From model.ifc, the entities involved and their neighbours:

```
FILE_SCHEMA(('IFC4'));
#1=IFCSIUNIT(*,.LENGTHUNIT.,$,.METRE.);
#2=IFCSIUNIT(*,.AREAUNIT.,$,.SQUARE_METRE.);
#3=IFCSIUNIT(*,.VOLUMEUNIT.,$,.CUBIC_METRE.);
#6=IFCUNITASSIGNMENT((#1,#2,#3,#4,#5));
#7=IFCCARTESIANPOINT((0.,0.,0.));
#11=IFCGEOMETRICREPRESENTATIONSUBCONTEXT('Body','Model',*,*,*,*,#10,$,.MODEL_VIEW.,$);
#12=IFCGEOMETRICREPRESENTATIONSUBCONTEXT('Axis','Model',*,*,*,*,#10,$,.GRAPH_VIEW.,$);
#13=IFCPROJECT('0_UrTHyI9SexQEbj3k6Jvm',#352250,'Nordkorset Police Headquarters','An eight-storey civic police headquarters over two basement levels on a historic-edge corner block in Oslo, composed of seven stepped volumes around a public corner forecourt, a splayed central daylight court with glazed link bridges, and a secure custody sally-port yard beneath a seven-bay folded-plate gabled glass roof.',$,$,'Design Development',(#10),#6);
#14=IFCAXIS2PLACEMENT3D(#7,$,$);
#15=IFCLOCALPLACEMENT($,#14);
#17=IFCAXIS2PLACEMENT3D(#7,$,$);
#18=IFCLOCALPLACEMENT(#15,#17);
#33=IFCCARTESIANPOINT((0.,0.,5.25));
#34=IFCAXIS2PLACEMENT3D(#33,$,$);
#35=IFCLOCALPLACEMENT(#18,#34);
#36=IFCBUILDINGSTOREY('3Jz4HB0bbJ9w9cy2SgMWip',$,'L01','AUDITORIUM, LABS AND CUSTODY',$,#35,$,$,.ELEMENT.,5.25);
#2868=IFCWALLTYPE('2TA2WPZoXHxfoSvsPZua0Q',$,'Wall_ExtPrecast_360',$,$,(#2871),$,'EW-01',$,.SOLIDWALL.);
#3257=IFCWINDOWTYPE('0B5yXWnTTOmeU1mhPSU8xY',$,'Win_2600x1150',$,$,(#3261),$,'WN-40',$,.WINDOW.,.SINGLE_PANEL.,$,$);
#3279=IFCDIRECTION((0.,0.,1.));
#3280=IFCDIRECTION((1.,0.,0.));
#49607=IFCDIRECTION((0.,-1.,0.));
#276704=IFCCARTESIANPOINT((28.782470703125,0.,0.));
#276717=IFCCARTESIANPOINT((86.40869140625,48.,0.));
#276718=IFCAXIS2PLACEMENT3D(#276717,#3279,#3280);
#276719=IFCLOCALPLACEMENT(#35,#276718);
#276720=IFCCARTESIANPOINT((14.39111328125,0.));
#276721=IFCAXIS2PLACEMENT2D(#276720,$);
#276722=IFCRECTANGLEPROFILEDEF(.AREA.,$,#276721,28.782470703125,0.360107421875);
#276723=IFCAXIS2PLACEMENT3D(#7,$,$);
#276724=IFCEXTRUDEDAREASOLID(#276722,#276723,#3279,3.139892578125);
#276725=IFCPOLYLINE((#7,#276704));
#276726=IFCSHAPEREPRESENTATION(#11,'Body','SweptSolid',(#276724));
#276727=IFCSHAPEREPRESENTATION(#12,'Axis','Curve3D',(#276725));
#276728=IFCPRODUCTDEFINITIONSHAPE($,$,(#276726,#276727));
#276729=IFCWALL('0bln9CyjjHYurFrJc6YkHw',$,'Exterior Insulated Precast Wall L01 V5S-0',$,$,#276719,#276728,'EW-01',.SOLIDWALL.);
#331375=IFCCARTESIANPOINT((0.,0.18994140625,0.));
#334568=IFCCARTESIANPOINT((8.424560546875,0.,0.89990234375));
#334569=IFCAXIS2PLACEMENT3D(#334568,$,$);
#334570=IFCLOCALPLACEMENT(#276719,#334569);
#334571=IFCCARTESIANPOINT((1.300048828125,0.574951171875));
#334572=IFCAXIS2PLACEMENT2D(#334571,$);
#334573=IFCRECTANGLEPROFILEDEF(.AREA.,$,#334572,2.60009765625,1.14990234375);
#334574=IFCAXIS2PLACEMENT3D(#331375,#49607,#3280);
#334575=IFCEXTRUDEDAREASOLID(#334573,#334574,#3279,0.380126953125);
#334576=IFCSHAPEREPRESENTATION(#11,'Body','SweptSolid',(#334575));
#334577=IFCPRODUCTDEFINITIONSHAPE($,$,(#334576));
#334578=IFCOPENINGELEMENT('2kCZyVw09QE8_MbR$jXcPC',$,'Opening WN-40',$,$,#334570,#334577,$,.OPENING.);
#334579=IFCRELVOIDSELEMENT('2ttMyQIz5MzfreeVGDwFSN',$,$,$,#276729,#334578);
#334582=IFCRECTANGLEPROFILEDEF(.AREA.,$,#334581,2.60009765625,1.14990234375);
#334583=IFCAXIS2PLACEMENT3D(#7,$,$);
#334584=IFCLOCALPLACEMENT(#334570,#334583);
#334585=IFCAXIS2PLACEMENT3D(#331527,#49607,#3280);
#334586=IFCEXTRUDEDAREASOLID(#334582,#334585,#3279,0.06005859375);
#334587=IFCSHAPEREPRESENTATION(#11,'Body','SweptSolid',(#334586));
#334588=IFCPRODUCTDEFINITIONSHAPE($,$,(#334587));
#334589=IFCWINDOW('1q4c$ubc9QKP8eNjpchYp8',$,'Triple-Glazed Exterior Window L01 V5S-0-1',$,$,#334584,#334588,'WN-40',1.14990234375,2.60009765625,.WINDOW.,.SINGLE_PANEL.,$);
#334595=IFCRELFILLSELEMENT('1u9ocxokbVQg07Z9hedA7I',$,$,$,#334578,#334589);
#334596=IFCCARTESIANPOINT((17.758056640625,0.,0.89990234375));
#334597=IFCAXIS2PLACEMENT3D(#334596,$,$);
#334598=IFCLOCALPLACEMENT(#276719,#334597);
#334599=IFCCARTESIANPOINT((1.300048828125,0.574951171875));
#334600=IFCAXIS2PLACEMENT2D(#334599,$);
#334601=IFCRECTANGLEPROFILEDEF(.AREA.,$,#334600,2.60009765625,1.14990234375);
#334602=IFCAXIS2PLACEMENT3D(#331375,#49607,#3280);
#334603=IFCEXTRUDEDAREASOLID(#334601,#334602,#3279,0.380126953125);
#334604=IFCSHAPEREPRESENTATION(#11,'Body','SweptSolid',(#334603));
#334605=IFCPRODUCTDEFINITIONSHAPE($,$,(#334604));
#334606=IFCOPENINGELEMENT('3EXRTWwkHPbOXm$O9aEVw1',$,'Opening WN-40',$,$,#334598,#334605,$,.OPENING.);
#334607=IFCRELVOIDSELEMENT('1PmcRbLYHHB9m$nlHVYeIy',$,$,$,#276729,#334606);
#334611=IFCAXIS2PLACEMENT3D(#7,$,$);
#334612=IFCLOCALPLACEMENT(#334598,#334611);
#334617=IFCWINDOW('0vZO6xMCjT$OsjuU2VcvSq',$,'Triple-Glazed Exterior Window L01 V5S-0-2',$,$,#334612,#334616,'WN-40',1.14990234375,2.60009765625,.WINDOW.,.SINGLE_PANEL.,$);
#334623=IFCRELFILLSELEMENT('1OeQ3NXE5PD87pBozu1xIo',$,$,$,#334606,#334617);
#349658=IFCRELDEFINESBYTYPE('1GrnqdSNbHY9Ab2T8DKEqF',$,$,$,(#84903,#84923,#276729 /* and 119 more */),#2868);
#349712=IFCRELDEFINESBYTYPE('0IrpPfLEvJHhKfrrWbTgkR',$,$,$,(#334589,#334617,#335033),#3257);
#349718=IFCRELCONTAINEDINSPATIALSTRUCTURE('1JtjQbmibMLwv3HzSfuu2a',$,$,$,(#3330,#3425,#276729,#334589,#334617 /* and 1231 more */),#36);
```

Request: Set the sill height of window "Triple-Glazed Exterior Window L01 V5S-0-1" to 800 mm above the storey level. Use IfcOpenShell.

```python
import numpy as np
import ifcopenshell
import ifcopenshell.api.geometry
import ifcopenshell.geom
import ifcopenshell.util.element
import ifcopenshell.util.placement
import ifcopenshell.util.shape
import ifcopenshell.util.unit

model = ifcopenshell.open("model.ifc")
unit_scale = ifcopenshell.util.unit.calculate_unit_scale(model)

window = model.by_guid("1q4c$ubc9QKP8eNjpchYp8")
opening = window.FillsVoids[0].RelatingOpeningElement
storey = ifcopenshell.util.element.get_container(window, ifc_class="IfcBuildingStorey")
level = ifcopenshell.util.placement.get_local_placement(storey.ObjectPlacement)[2, 3]

# The opening's origin need not be at the sill, so measure its lowest point.
shape = ifcopenshell.geom.create_shape(ifcopenshell.geom.settings(), opening)
bottom = ifcopenshell.util.shape.get_shape_bottom_elevation(shape, shape.geometry) / unit_scale
dz = level + 0.8 / unit_scale - bottom

shift = np.array([0.0, 0.0, dz])
# The window is placed relative to its opening, so it follows when the opening moves.
matrix = ifcopenshell.util.placement.get_local_placement(opening.ObjectPlacement)
matrix[:3, 3] += shift
ifcopenshell.api.geometry.edit_object_placement(
    model, product=opening, matrix=matrix, is_si=False, should_transform_children=True
)

print(f"moved by {dz * unit_scale:+.3f} m")

model.write("model-out.ifc")
```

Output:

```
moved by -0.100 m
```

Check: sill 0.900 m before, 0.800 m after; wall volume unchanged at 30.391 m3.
